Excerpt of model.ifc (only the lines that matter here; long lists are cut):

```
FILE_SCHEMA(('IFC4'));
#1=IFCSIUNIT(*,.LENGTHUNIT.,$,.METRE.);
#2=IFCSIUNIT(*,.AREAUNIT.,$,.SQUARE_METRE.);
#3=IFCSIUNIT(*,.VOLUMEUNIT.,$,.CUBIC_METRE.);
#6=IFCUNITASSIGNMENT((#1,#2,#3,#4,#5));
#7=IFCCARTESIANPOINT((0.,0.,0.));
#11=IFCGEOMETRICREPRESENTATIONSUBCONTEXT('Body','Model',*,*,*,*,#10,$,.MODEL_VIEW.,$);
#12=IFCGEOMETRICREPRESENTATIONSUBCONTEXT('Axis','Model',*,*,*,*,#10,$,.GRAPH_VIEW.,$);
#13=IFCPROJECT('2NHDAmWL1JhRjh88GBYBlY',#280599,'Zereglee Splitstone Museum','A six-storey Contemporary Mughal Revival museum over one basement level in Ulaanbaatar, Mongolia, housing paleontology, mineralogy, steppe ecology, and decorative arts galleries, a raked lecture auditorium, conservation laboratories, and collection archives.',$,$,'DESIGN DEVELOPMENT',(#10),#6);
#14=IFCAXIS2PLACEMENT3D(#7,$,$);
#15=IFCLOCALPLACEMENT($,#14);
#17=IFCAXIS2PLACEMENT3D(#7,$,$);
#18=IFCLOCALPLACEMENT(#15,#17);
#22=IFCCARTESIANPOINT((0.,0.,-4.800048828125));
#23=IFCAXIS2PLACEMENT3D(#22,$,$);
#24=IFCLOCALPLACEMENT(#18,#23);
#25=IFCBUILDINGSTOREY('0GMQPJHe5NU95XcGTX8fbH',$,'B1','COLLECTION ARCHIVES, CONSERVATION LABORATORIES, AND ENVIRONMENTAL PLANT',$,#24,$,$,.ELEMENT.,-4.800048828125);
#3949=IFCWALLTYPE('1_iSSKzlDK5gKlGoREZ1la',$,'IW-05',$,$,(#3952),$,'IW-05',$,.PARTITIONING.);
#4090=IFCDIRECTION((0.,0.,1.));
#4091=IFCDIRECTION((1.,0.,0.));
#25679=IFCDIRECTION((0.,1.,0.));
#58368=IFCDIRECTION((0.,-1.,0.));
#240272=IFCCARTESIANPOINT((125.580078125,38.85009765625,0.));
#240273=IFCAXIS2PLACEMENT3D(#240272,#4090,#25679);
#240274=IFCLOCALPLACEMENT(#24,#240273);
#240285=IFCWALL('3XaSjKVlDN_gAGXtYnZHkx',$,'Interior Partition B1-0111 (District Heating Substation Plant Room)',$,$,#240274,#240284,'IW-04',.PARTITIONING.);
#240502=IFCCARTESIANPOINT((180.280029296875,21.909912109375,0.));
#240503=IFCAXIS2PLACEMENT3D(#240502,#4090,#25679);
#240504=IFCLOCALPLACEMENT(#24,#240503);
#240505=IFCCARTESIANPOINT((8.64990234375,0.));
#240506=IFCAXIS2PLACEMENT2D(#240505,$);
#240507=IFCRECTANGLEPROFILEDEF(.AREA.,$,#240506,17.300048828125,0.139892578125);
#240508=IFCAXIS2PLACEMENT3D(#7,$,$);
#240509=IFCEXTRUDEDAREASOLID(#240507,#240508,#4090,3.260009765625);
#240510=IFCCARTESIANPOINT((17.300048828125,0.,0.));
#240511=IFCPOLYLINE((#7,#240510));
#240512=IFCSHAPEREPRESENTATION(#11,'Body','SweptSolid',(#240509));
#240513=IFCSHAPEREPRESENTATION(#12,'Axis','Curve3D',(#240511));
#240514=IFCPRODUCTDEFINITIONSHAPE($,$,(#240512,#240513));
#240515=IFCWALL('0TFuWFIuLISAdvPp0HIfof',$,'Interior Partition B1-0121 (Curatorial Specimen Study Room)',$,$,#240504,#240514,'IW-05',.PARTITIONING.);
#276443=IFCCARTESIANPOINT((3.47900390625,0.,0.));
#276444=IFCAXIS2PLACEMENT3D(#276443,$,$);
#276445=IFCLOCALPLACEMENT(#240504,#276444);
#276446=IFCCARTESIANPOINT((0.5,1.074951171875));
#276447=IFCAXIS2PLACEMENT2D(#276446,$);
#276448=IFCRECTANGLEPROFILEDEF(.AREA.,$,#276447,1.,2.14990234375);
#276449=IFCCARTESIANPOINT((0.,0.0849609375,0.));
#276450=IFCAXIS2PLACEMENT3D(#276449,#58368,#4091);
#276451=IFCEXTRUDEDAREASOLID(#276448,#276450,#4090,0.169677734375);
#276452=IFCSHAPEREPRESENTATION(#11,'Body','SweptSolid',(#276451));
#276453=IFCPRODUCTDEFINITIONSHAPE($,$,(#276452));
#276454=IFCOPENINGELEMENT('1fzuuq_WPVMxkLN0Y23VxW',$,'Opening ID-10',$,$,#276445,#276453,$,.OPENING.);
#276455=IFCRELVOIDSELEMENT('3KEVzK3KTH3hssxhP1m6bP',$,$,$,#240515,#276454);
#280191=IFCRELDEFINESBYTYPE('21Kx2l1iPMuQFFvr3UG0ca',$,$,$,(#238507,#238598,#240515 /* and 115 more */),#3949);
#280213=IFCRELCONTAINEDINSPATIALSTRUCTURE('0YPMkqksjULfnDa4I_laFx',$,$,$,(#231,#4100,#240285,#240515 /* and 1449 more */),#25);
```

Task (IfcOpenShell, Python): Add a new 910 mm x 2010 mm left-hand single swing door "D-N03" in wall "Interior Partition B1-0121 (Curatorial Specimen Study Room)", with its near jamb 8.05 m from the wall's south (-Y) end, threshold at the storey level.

```python
import numpy as np
import ifcopenshell
import ifcopenshell.api.feature
import ifcopenshell.api.geometry
import ifcopenshell.api.root
import ifcopenshell.api.spatial
import ifcopenshell.geom
import ifcopenshell.util.element
import ifcopenshell.util.placement
import ifcopenshell.util.representation
import ifcopenshell.util.shape
import ifcopenshell.util.unit

model = ifcopenshell.open("model.ifc")
unit_scale = ifcopenshell.util.unit.calculate_unit_scale(model)
settings = ifcopenshell.geom.settings()


def volume(element):
    """Net volume in cubic metres, openings subtracted."""
    shape = ifcopenshell.geom.create_shape(settings, element)
    return ifcopenshell.util.shape.get_volume(shape.geometry)


wall = model.by_id(240515)
storey = ifcopenshell.util.element.get_container(wall, ifc_class="IfcBuildingStorey")
context = ifcopenshell.util.representation.get_context(model, "Model", "Body", "MODEL_VIEW")
before = volume(wall)

width, height, from_end, sill = 0.91, 2.01, 8.05, 0.0  # metres

# The wall runs along its own X axis, and the end named is its -X end.
wall_shape = ifcopenshell.geom.create_shape(settings, wall)
x, y, z = ifcopenshell.util.shape.get_vertices(wall_shape.geometry).T
start = x.min() + from_end
face, thickness = float(y.min()), float(y.max() - y.min())
wall_matrix = ifcopenshell.util.placement.get_local_placement(wall.ObjectPlacement)
level = ifcopenshell.util.placement.get_local_placement(storey.ObjectPlacement)[2, 3]


def in_wall(x, y):
    """Placement at x, y metres in the wall's axes, at sill height."""
    matrix = wall_matrix.copy()
    matrix[:, 3] = wall_matrix @ np.array([x / unit_scale, y / unit_scale, 0.0, 1.0])
    matrix[2, 3] = level + sill / unit_scale
    return matrix


# Opening: a box that overshoots both wall faces by 50 mm.
opening = ifcopenshell.api.root.create_entity(model, ifc_class="IfcOpeningElement", predefined_type="OPENING")
box = ifcopenshell.api.geometry.add_wall_representation(
    model, context=context, length=width, height=height, thickness=thickness + 0.1
)
ifcopenshell.api.geometry.assign_representation(model, product=opening, representation=box)
ifcopenshell.api.geometry.edit_object_placement(model, product=opening, matrix=in_wall(start, face - 0.05), is_si=False)
ifcopenshell.api.feature.add_feature(model, feature=opening, element=wall)

door = ifcopenshell.api.root.create_entity(model, ifc_class="IfcDoor", name="D-N03", predefined_type="DOOR")
door.OverallWidth, door.OverallHeight = width / unit_scale, height / unit_scale
door.OperationType = "SINGLE_SWING_LEFT"
body = ifcopenshell.api.geometry.add_door_representation(
    model,
    context=context,
    overall_width=door.OverallWidth,
    overall_height=door.OverallHeight,
    operation_type="SINGLE_SWING_LEFT",
    lining_properties={"LiningDepth": thickness / unit_scale, "ThresholdDepth": thickness / unit_scale},
)
ifcopenshell.api.geometry.assign_representation(model, product=door, representation=body)
ifcopenshell.api.spatial.assign_container(model, products=[door], relating_structure=storey)
ifcopenshell.api.feature.add_filling(model, opening=opening, element=door)

# The lining spans the wall, so the door starts at the wall face.
ifcopenshell.api.geometry.edit_object_placement(model, product=door, matrix=in_wall(start, face), is_si=False)

after = volume(wall)

print(f"wall volume {before:.3f} -> {after:.3f} m3")

model.write("model-out.ifc")
```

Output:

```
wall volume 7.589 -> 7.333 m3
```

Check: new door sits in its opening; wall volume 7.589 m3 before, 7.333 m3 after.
